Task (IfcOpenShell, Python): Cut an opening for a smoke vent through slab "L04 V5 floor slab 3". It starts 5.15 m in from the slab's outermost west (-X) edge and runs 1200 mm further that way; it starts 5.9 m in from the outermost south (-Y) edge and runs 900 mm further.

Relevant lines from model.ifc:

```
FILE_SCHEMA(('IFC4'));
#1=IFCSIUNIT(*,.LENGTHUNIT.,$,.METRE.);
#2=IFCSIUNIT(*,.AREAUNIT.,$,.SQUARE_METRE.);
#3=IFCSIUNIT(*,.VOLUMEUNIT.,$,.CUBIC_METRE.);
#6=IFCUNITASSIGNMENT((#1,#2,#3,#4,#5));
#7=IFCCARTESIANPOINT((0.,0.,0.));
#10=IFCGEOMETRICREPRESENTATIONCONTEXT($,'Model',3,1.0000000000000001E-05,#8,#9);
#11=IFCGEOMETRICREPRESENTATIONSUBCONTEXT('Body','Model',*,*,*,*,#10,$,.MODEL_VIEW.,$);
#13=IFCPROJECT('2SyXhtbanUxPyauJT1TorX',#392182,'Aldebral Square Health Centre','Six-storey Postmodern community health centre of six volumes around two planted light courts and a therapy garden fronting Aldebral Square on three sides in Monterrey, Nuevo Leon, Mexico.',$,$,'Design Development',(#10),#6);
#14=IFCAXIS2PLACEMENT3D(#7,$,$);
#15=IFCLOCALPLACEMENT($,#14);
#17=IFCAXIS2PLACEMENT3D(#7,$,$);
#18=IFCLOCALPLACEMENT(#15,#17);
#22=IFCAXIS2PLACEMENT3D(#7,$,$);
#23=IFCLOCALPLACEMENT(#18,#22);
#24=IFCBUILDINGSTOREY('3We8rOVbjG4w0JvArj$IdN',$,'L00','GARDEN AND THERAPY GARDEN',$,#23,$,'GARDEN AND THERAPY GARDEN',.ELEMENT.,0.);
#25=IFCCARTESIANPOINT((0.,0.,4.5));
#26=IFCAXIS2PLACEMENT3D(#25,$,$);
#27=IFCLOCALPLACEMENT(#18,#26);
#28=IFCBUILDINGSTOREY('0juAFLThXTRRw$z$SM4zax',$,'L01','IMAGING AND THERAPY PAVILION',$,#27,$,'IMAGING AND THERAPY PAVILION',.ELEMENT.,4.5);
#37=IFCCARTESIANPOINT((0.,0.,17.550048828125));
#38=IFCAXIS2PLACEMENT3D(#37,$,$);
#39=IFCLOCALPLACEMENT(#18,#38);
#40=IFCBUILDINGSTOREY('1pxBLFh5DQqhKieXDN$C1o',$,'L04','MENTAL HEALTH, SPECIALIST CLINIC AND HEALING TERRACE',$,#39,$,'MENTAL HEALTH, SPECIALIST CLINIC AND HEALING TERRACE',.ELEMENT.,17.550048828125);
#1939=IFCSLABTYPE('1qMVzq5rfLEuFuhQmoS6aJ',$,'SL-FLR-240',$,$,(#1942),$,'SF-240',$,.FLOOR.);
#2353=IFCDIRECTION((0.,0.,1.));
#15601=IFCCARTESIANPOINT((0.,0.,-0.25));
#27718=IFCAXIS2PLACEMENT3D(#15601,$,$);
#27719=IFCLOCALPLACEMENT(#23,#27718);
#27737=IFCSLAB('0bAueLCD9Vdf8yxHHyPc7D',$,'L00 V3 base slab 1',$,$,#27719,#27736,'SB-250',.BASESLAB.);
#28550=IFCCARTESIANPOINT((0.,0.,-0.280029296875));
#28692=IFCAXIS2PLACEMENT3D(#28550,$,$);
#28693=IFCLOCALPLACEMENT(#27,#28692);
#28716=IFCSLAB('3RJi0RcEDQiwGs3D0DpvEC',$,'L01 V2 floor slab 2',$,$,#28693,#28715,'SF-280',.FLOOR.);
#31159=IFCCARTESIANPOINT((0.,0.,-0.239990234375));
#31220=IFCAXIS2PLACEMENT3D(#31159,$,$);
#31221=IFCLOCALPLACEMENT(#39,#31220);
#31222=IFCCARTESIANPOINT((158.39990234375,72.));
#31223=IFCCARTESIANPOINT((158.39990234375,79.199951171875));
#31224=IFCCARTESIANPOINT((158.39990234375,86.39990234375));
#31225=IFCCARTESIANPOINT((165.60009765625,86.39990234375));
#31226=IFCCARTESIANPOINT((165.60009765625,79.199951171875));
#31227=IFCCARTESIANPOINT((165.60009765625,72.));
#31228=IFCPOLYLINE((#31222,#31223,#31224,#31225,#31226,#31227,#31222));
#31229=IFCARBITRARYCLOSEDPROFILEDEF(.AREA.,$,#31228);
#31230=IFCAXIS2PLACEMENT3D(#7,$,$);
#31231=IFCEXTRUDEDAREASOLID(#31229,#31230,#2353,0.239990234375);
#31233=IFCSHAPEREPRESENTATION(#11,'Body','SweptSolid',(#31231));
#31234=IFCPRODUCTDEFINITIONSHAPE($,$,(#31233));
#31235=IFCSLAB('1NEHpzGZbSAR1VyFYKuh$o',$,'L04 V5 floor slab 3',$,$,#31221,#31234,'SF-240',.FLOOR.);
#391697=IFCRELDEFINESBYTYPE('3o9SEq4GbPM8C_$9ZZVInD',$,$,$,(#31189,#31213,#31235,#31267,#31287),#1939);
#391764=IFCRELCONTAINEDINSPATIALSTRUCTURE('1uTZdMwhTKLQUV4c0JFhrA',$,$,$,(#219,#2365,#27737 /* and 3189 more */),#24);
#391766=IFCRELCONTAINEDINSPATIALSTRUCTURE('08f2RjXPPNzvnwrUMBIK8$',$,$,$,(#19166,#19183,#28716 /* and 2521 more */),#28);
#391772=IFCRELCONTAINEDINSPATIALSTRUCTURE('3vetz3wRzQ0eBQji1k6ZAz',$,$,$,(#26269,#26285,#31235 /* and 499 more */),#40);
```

```python
import numpy as np
import ifcopenshell
import ifcopenshell.api.feature
import ifcopenshell.api.geometry
import ifcopenshell.api.root
import ifcopenshell.geom
import ifcopenshell.util.placement
import ifcopenshell.util.representation
import ifcopenshell.util.shape
import ifcopenshell.util.unit

model = ifcopenshell.open("model.ifc")
unit_scale = ifcopenshell.util.unit.calculate_unit_scale(model)
settings = ifcopenshell.geom.settings()


def volume(element):
    """Net volume in cubic metres, openings subtracted."""
    shape = ifcopenshell.geom.create_shape(settings, element)
    return ifcopenshell.util.shape.get_volume(shape.geometry)


slab = model.by_id(31235)
before = volume(slab)

# Extent in the slab's own axes, in metres. The edges named are its -X and -Y sides.
slab_shape = ifcopenshell.geom.create_shape(settings, slab)
vertices = ifcopenshell.util.shape.get_vertices(slab_shape.geometry)
x_min, y_min, bottom = vertices.min(axis=0)
top = vertices[:, 2].max()

opening = ifcopenshell.api.root.create_entity(model, ifc_class="IfcOpeningElement", name="Smoke vent opening", predefined_type="OPENING")
context = ifcopenshell.util.representation.get_context(model, "Model", "Body", "MODEL_VIEW")
width, depth = 1.2, 0.9
outline = [(0.0, 0.0), (width, 0.0), (width, depth), (0.0, depth), (0.0, 0.0)]
# Overshoot both faces by 50 mm so the cut is clean.
shape = ifcopenshell.api.geometry.add_slab_representation(
    model, context=context, depth=top - bottom + 0.1, polyline=outline
)
ifcopenshell.api.geometry.assign_representation(model, product=opening, representation=shape)

matrix = ifcopenshell.util.placement.get_local_placement(slab.ObjectPlacement)
matrix[:, 3] = matrix @ np.append(np.array([x_min + 5.15, y_min + 5.9, bottom - 0.05]) / unit_scale, 1.0)
ifcopenshell.api.geometry.edit_object_placement(model, product=opening, matrix=matrix, is_si=False)
ifcopenshell.api.feature.add_feature(model, feature=opening, element=slab)

after = volume(slab)

print(f"slab volume {before:.3f} -> {after:.3f} m3")

model.write("model_rev.ifc")
```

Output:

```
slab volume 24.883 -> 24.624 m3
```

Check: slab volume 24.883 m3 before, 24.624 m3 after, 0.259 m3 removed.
